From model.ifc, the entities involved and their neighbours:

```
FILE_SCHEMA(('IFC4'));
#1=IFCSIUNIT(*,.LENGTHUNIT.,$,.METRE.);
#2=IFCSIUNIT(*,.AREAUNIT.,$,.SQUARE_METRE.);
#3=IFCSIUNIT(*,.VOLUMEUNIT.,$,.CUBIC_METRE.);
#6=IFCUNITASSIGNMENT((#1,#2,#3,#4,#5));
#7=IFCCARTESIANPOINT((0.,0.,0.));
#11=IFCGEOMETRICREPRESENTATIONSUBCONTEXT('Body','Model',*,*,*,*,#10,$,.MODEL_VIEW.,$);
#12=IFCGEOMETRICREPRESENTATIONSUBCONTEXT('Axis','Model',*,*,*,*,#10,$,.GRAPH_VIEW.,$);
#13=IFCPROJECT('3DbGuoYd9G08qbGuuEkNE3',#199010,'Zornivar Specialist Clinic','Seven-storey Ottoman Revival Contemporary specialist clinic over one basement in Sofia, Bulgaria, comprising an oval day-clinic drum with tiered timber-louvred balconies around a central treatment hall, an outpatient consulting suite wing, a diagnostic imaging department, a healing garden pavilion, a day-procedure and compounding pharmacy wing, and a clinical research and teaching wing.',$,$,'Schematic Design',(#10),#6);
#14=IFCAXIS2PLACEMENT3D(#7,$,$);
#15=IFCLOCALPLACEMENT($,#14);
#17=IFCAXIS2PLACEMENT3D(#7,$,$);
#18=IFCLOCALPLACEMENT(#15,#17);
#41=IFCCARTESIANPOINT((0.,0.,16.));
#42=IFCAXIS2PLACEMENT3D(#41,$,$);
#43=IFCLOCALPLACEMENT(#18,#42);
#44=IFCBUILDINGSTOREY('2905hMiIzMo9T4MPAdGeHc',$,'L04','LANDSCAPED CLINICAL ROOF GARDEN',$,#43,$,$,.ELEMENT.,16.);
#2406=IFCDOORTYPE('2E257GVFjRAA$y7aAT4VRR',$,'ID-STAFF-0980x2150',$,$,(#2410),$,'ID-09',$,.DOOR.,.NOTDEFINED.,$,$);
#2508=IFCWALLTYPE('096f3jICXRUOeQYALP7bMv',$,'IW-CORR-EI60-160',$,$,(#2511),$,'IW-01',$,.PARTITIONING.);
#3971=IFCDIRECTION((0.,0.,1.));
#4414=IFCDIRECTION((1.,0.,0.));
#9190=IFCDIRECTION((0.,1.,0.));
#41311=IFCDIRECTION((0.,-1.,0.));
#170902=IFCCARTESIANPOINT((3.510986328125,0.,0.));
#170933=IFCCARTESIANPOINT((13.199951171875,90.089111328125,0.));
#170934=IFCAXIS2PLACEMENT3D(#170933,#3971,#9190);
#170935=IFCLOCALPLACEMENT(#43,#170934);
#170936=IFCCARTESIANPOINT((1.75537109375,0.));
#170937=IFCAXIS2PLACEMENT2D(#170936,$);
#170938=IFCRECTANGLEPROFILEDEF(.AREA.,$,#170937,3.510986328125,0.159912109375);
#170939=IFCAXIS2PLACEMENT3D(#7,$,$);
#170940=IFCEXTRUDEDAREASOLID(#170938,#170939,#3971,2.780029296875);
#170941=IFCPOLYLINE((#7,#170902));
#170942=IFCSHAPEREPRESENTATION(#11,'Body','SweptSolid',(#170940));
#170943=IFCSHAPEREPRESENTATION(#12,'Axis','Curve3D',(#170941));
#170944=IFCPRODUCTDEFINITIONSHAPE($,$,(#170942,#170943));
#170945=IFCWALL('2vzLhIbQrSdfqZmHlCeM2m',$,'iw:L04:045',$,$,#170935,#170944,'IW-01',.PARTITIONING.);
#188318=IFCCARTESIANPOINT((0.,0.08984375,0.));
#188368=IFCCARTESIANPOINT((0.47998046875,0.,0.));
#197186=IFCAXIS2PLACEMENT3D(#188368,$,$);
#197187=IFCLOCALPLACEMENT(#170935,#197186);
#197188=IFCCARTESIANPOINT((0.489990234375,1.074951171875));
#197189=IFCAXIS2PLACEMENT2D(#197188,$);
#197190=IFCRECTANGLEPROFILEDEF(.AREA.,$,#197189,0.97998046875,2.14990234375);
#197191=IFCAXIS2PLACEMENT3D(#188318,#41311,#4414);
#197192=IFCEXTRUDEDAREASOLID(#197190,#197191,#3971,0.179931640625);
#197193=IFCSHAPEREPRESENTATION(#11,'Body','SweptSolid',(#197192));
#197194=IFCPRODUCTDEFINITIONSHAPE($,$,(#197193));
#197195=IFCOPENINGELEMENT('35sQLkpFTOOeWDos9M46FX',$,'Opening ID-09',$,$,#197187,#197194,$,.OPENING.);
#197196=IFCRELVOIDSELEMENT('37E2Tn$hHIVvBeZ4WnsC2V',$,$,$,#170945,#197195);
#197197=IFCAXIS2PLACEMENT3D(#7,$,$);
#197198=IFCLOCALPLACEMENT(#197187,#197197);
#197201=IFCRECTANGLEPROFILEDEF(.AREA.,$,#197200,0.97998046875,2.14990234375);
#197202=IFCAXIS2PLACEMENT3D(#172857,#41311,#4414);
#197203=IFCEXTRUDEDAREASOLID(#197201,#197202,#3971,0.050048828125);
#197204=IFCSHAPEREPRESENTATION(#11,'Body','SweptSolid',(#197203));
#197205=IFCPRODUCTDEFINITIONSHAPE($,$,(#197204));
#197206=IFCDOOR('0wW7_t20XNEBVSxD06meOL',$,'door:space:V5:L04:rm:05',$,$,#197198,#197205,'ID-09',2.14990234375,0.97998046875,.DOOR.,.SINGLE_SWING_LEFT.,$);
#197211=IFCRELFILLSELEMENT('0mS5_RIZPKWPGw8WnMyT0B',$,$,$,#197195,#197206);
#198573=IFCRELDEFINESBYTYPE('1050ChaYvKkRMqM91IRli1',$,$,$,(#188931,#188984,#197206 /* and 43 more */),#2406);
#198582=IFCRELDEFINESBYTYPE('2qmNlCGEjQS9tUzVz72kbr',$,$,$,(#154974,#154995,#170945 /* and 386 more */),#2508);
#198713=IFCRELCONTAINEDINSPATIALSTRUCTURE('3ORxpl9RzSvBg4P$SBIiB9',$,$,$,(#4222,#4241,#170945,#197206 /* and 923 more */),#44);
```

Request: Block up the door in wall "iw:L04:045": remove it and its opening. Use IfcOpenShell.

```python
import ifcopenshell
import ifcopenshell.api.feature
import ifcopenshell.api.root
import ifcopenshell.geom
import ifcopenshell.util.shape

model = ifcopenshell.open("model.ifc")
settings = ifcopenshell.geom.settings()


def volume(element):
    """Net volume in cubic metres, openings subtracted."""
    shape = ifcopenshell.geom.create_shape(settings, element)
    return ifcopenshell.util.shape.get_volume(shape.geometry)


door = model.by_guid("0wW7_t20XNEBVSxD06meOL")
opening = door.FillsVoids[0].RelatingOpeningElement
wall = opening.VoidsElements[0].RelatingBuildingElement
before = volume(wall)

ifcopenshell.api.root.remove_product(model, product=door)
ifcopenshell.api.feature.remove_feature(model, feature=opening)

after = volume(wall)

print(f"wall volume {before:.3f} -> {after:.3f} m3")

model.write("model-out.ifc")
```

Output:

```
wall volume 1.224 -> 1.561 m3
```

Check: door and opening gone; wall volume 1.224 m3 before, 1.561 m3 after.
